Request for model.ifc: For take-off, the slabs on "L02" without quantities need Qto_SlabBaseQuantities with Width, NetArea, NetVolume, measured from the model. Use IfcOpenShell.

First a look at what the model holds.

```python
import ifcopenshell
import ifcopenshell.util.element
import ifcopenshell.util.unit

model = ifcopenshell.open("model.ifc")
print(model.schema)
for unit_type in ("LENGTHUNIT", "AREAUNIT", "VOLUMEUNIT"):
    print(unit_type, ifcopenshell.util.unit.calculate_unit_scale(model, unit_type))
storey = next(s for s in model.by_type("IfcBuildingStorey") if s.Name == "L02")
slabs = [e for e in ifcopenshell.util.element.get_decomposition(storey) if e.is_a("IfcSlab")]
for e in sorted(slabs, key=lambda e: e.id()):
    print(e.id(), e.is_a(), e.Name, list(ifcopenshell.util.element.get_psets(e, qtos_only=True)), sep=" | ")
```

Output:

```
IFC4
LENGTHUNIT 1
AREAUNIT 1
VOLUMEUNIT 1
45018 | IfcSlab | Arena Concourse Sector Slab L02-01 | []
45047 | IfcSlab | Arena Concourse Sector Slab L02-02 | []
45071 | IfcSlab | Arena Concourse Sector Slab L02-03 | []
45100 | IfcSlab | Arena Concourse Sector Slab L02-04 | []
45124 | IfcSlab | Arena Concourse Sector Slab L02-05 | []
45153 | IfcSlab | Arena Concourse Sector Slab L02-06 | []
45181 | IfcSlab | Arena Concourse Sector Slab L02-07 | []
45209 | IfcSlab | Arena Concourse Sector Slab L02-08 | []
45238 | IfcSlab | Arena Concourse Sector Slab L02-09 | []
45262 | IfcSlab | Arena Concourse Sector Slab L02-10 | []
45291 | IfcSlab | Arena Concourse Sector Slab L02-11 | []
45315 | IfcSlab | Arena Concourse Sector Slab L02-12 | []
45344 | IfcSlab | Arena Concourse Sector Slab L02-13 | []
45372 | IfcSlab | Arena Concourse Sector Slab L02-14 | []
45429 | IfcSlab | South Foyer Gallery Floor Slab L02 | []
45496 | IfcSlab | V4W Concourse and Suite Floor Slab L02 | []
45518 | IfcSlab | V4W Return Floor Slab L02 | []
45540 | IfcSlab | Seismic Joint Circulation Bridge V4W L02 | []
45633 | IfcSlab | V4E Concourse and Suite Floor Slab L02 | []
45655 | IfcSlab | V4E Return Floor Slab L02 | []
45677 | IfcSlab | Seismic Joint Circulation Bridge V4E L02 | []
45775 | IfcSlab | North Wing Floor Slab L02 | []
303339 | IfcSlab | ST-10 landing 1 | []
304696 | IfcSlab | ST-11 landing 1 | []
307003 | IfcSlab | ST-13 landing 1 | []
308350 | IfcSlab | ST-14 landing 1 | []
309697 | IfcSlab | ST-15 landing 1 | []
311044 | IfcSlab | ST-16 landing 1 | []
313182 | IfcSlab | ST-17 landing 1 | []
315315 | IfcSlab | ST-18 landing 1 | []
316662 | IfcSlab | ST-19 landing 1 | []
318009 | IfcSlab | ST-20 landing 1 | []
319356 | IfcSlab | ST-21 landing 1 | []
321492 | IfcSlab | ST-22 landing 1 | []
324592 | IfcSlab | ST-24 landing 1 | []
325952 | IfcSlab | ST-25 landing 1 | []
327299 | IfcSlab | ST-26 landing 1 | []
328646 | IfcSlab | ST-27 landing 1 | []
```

```python
import ifcopenshell
import ifcopenshell.api.pset
import ifcopenshell.geom
import ifcopenshell.util.element
import ifcopenshell.util.shape
import ifcopenshell.util.unit

model = ifcopenshell.open("model.ifc")
unit_scale = ifcopenshell.util.unit.calculate_unit_scale(model)
area_scale = ifcopenshell.util.unit.calculate_unit_scale(model, "AREAUNIT")
volume_scale = ifcopenshell.util.unit.calculate_unit_scale(model, "VOLUMEUNIT")
settings = ifcopenshell.geom.settings()

storey = next(s for s in model.by_type("IfcBuildingStorey") if s.Name == "L02")
slabs = [e for e in ifcopenshell.util.element.get_decomposition(storey) if e.is_a("IfcSlab")]

for e in sorted(slabs, key=lambda e: e.id()):
    if ifcopenshell.util.element.get_psets(e, qtos_only=True, should_inherit=False):
        continue
    # Geometry comes back in metres, in the element's own axes.
    shape = ifcopenshell.geom.create_shape(settings, e)
    values = {
        "Width": ifcopenshell.util.shape.get_z(shape.geometry) / unit_scale,
        "NetArea": ifcopenshell.util.shape.get_footprint_area(shape.geometry) / area_scale,
        "NetVolume": ifcopenshell.util.shape.get_volume(shape.geometry) / volume_scale,
    }
    qto = ifcopenshell.api.pset.add_qto(model, product=e, name="Qto_SlabBaseQuantities")
    ifcopenshell.api.pset.edit_qto(model, qto=qto, properties=values)
    print(e.id(), {k: round(v, 3) for k, v in values.items()})

model.write("model_rev.ifc")
```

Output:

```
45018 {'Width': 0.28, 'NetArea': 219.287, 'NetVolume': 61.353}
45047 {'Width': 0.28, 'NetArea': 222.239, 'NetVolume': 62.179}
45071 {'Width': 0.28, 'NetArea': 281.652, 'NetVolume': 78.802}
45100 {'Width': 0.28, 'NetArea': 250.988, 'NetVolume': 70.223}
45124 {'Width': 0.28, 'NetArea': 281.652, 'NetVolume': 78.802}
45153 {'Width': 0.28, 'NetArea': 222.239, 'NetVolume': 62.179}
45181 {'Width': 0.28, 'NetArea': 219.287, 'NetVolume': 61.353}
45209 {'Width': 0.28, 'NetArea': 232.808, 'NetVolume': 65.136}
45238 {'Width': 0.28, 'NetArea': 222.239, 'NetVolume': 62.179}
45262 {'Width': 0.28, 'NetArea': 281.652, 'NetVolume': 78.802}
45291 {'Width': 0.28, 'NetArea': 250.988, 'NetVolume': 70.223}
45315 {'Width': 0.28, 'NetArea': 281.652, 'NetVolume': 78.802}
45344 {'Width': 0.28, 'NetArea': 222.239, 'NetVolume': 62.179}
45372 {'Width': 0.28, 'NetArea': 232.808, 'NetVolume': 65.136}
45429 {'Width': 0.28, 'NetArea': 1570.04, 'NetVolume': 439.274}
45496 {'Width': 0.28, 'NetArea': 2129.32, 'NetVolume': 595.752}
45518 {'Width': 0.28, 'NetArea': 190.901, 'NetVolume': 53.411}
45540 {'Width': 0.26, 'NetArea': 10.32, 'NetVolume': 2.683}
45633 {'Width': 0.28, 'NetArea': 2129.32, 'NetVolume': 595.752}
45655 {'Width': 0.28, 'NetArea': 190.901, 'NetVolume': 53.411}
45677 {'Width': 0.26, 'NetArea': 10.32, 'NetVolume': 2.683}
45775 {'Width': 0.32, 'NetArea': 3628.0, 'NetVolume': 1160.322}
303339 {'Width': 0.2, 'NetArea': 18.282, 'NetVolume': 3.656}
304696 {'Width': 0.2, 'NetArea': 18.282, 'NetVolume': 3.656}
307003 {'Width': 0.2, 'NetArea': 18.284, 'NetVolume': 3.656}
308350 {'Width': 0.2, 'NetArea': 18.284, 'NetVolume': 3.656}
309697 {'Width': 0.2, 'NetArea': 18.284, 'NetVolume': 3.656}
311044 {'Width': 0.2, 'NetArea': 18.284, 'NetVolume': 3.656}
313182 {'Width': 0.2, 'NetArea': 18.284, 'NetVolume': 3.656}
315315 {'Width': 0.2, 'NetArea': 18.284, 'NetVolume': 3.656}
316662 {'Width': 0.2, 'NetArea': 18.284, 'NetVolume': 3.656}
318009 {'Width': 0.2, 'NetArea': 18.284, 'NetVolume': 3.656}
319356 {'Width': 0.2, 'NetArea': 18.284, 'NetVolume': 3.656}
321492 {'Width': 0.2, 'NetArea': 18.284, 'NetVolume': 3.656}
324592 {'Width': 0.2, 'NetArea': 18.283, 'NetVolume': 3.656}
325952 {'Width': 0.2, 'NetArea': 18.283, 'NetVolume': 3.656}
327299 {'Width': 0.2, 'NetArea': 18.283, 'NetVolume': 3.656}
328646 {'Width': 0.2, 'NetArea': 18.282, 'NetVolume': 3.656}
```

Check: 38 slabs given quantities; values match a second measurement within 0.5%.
